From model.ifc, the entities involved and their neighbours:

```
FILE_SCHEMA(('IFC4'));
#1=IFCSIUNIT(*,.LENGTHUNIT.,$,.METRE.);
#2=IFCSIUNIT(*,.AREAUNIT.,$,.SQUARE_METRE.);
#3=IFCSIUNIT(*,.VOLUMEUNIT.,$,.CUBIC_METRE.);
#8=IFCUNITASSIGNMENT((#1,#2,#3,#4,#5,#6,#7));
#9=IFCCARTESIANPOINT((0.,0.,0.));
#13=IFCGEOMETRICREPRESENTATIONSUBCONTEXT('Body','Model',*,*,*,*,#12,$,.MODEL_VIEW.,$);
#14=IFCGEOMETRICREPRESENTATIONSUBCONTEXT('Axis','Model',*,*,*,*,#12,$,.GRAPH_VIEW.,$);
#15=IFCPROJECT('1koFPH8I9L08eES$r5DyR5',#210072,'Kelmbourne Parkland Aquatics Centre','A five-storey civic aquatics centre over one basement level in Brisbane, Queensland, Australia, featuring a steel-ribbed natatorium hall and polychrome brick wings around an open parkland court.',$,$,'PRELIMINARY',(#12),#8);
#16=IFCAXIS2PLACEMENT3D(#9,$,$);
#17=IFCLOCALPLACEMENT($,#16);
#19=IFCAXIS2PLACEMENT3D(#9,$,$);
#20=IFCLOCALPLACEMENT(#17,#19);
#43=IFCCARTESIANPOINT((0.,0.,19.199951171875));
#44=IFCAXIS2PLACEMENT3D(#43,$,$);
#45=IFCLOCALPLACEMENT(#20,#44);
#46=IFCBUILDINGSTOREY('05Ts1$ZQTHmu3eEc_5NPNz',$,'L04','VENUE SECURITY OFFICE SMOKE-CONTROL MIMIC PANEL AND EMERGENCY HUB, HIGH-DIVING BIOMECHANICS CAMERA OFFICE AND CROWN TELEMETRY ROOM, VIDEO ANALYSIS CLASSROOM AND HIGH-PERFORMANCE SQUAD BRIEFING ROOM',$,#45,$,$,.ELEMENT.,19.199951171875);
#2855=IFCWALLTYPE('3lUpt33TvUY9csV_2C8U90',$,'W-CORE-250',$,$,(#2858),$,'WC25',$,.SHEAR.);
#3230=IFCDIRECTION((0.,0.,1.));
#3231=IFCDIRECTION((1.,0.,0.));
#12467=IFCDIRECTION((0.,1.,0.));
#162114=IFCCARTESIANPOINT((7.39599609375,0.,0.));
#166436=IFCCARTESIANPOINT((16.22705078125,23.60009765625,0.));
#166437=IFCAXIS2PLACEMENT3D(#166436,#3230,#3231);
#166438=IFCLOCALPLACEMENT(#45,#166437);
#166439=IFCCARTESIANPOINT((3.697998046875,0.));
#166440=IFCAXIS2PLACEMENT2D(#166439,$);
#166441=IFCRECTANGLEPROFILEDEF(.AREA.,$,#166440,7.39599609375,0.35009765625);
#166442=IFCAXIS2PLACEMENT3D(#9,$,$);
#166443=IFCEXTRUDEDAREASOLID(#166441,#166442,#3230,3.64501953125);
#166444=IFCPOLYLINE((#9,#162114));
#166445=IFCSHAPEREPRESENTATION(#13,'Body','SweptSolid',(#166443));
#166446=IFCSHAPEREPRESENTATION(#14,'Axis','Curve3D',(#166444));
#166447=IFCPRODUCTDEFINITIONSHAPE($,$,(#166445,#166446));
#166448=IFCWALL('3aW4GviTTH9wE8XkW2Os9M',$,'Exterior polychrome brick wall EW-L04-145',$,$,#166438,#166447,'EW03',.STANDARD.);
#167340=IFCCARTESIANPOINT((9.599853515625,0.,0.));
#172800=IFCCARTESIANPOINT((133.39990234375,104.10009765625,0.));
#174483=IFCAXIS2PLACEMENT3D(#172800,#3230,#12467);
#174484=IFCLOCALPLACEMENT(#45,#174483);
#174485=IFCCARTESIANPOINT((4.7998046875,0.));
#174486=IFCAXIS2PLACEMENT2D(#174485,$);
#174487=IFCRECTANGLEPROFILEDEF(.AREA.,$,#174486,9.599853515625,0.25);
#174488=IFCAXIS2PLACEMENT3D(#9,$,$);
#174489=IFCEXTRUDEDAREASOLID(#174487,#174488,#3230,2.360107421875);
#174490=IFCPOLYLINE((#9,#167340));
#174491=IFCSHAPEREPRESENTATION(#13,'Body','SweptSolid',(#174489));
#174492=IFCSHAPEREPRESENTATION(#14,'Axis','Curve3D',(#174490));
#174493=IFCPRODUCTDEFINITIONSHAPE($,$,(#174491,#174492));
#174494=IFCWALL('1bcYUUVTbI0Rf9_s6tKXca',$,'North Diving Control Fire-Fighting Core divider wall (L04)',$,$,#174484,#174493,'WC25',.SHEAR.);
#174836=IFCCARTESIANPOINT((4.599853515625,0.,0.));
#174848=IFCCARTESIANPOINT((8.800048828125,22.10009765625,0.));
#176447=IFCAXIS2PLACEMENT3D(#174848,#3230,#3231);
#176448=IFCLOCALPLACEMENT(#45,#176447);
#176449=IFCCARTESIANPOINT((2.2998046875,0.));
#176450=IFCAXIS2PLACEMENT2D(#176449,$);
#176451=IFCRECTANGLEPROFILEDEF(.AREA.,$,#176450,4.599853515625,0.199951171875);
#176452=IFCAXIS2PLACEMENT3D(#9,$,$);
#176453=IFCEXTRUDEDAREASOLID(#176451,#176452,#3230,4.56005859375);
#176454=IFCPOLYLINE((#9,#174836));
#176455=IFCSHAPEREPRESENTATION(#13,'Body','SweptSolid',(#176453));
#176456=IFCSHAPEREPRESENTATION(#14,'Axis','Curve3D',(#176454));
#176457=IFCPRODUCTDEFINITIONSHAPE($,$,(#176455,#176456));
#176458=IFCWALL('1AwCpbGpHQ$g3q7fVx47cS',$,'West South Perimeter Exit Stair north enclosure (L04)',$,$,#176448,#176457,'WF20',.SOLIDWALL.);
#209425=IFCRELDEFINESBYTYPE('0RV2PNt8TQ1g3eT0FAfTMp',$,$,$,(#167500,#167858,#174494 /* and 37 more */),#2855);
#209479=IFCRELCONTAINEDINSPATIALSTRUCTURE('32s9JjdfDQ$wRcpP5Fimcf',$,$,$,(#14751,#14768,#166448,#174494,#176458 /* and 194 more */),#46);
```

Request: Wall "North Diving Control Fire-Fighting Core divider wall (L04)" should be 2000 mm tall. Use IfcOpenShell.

```python
import ifcopenshell
import ifcopenshell.geom
import ifcopenshell.util.representation
import ifcopenshell.util.shape
import ifcopenshell.util.unit

model = ifcopenshell.open("model.ifc")
unit_scale = ifcopenshell.util.unit.calculate_unit_scale(model)
settings = ifcopenshell.geom.settings()


def volume(element):
    """Net volume in cubic metres, openings subtracted."""
    shape = ifcopenshell.geom.create_shape(settings, element)
    return ifcopenshell.util.shape.get_volume(shape.geometry)


wall = model.by_guid("1bcYUUVTbI0Rf9_s6tKXca")
before = volume(wall)

body = ifcopenshell.util.representation.get_representation(wall, "Model", "Body")
solid = body.Items[0]
old_height = solid.Depth
solid.Depth = 2 / unit_scale
after = volume(wall)

print(f"height {old_height:g} -> {solid.Depth:g}, volume {before:.3f} -> {after:.3f} m3")

model.write("model_v2.ifc")
```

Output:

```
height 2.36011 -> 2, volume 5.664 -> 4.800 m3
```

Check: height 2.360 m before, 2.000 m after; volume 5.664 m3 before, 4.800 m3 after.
